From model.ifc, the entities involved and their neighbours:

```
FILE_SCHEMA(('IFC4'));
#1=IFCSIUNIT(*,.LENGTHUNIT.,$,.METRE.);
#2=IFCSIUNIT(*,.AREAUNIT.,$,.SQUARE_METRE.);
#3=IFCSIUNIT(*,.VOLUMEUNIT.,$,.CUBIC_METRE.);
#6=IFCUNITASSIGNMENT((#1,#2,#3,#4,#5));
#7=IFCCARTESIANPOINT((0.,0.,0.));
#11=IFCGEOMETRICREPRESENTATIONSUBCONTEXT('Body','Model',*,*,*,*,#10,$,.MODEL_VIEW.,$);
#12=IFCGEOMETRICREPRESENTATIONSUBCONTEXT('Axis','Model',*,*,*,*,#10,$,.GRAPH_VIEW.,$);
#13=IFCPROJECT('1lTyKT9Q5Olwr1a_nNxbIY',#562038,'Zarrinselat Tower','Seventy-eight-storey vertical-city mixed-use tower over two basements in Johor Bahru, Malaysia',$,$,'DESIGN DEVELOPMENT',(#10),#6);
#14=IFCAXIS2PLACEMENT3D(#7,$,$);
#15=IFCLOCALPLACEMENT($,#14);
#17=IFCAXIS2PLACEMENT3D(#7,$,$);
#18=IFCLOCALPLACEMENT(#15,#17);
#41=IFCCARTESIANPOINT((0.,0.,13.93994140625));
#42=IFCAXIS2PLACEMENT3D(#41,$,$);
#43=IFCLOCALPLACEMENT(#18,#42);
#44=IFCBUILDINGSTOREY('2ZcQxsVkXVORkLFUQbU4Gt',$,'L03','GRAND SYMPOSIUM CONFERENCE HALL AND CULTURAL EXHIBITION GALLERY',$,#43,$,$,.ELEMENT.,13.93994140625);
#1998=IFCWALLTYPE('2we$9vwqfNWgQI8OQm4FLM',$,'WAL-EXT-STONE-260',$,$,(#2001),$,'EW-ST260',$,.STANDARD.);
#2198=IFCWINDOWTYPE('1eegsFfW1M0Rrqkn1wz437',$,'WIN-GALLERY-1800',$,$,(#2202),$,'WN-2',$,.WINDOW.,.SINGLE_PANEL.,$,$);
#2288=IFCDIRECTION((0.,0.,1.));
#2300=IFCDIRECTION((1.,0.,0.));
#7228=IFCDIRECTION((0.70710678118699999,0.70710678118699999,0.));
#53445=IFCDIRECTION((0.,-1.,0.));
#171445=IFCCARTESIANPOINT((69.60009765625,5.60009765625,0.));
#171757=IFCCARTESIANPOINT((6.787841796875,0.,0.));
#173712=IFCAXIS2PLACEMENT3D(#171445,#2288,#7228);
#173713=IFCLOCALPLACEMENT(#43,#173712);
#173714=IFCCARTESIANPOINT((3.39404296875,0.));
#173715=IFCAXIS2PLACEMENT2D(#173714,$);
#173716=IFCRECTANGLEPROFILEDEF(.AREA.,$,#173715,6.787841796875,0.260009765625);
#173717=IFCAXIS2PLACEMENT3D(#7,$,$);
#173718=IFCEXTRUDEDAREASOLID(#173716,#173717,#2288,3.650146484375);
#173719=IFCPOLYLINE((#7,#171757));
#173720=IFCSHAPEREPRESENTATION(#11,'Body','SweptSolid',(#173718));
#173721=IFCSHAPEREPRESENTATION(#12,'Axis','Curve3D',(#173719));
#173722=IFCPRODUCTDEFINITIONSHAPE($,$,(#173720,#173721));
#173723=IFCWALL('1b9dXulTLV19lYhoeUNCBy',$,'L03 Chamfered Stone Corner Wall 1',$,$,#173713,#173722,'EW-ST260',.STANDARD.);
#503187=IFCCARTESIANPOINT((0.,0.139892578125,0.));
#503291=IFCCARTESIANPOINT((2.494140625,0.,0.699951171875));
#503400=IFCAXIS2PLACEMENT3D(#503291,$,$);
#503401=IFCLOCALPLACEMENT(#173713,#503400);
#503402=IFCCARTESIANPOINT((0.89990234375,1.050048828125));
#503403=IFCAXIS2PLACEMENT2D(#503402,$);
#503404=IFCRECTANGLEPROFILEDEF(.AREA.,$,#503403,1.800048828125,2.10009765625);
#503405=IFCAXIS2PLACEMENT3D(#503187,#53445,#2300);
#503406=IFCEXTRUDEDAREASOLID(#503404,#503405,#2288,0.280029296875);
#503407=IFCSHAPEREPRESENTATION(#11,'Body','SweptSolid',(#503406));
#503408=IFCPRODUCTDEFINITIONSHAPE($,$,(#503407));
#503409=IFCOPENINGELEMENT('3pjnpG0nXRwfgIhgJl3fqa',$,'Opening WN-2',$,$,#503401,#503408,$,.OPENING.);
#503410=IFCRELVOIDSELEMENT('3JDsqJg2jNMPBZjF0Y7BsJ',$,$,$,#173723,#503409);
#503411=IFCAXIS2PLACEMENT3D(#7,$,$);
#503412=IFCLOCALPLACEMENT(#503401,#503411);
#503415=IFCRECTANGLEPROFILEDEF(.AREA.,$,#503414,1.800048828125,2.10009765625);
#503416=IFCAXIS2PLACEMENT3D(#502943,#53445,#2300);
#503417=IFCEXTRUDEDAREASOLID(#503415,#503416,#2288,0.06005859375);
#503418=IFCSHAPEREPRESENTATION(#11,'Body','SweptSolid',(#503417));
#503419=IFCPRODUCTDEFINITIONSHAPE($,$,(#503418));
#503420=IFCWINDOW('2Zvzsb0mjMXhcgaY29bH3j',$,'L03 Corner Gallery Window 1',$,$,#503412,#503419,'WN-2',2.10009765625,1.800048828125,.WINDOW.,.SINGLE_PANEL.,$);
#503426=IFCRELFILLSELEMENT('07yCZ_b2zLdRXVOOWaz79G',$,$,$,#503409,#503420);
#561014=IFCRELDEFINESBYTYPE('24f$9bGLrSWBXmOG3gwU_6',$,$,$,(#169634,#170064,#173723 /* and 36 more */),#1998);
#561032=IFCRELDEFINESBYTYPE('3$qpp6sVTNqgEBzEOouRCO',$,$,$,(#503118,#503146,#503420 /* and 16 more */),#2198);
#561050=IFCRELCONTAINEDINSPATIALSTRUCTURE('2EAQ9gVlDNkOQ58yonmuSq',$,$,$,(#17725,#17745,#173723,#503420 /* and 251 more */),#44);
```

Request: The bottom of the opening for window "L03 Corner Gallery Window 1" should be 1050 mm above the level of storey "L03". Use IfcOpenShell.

```python
import numpy as np
import ifcopenshell
import ifcopenshell.api.geometry
import ifcopenshell.geom
import ifcopenshell.util.element
import ifcopenshell.util.placement
import ifcopenshell.util.shape
import ifcopenshell.util.unit

model = ifcopenshell.open("model.ifc")
unit_scale = ifcopenshell.util.unit.calculate_unit_scale(model)

window = model.by_id(503420)
opening = window.FillsVoids[0].RelatingOpeningElement
storey = ifcopenshell.util.element.get_container(window, ifc_class="IfcBuildingStorey")
level = ifcopenshell.util.placement.get_local_placement(storey.ObjectPlacement)[2, 3]

# The opening's origin need not be at the sill, so measure its lowest point.
shape = ifcopenshell.geom.create_shape(ifcopenshell.geom.settings(), opening)
bottom = ifcopenshell.util.shape.get_shape_bottom_elevation(shape, shape.geometry) / unit_scale
dz = level + 1.05 / unit_scale - bottom

shift = np.array([0.0, 0.0, dz])
# The window is placed relative to its opening, so it follows when the opening moves.
matrix = ifcopenshell.util.placement.get_local_placement(opening.ObjectPlacement)
matrix[:3, 3] += shift
ifcopenshell.api.geometry.edit_object_placement(
    model, product=opening, matrix=matrix, is_si=False, should_transform_children=True
)

print(f"moved by {dz * unit_scale:+.3f} m")

model.write("model-out.ifc")
```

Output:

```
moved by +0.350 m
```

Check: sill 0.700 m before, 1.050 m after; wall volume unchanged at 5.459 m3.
